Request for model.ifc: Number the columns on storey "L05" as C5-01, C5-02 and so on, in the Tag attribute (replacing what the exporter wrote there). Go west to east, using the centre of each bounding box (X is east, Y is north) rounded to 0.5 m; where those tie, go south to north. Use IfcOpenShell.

First a look at what the model holds.

```python
import ifcopenshell
import ifcopenshell.util.element
import ifcopenshell.util.placement

model = ifcopenshell.open("model.ifc")
print(model.schema)
storey = next(s for s in model.by_type("IfcBuildingStorey") if s.Name == "L05")
columns = [e for e in ifcopenshell.util.element.get_decomposition(storey) if e.is_a("IfcColumn")]
for e in sorted(columns, key=lambda e: e.id()):
    origin = ifcopenshell.util.placement.get_local_placement(e.ObjectPlacement)[:3, 3]
    print(e.id(), e.Tag, e.Name, origin.round(2) + 0.0, sep=" | ")
```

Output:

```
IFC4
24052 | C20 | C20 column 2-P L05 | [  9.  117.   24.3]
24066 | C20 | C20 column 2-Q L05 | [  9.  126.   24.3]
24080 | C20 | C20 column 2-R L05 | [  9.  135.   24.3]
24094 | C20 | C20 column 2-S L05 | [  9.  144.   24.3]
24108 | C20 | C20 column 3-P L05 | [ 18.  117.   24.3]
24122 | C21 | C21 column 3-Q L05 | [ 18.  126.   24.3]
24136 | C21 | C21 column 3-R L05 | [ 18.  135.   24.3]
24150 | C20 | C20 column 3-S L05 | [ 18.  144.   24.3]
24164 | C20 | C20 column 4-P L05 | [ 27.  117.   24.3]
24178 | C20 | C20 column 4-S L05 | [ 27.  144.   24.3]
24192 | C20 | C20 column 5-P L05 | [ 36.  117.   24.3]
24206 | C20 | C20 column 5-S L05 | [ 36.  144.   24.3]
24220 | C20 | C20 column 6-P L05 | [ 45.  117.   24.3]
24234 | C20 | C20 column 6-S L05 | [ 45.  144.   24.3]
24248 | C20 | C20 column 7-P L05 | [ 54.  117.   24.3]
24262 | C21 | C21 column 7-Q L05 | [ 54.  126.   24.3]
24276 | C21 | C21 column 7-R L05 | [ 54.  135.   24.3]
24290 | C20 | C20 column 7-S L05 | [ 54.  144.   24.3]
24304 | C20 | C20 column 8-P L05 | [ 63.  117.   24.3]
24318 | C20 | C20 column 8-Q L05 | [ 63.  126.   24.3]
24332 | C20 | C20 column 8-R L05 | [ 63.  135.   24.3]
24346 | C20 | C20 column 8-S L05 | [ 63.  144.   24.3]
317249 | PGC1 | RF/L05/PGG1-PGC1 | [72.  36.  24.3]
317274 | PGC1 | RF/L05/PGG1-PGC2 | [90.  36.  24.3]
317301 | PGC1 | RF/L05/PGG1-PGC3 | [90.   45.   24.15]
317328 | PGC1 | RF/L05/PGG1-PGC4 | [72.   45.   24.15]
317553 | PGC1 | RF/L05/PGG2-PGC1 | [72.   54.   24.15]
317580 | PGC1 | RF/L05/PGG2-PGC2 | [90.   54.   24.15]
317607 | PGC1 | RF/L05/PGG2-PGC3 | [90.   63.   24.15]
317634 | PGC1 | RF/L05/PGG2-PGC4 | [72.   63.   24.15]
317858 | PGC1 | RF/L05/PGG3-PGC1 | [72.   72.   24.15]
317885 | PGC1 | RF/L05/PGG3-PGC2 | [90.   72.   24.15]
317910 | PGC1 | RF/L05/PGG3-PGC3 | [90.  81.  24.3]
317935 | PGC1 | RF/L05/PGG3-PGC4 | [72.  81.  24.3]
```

```python
import ifcopenshell
import ifcopenshell.geom
import ifcopenshell.util.element
import ifcopenshell.util.shape

model = ifcopenshell.open("model.ifc")
settings = ifcopenshell.geom.settings()
settings.set("use-world-coords", True)


def centre(element):
    shape = ifcopenshell.geom.create_shape(settings, element)
    return ifcopenshell.util.shape.get_bbox_centroid(shape.geometry)


storey = next(s for s in model.by_type("IfcBuildingStorey") if s.Name == "L05")
columns = [e for e in ifcopenshell.util.element.get_decomposition(storey) if e.is_a("IfcColumn")]

# Insertion points can sit at a corner or the storey origin, so sort by the geometry (in metres).
centres = {e: centre(e) for e in columns}
columns.sort(key=lambda e: (round(centres[e][0] / 0.5), centres[e][1]))

for i, e in enumerate(columns, start=1):
    number = f"C5-{i:02d}"
    e.Tag = number
    print(e.id(), number)

model.write("model_edited.ifc")
```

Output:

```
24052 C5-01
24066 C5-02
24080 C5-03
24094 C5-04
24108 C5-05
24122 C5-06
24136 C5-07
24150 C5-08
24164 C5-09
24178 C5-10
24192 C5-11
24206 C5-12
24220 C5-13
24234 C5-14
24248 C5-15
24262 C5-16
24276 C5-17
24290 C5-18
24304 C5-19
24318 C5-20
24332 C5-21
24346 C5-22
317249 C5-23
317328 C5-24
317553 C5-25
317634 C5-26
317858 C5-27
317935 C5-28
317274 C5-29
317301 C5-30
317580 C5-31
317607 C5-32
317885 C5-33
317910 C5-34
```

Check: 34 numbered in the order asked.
